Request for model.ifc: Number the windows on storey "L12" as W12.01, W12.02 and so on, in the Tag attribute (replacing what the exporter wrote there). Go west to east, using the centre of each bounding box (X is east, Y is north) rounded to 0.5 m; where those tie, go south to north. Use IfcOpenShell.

First a look at what the model holds.

```python
import ifcopenshell
import ifcopenshell.util.element
import ifcopenshell.util.placement

model = ifcopenshell.open("model.ifc")
print(model.schema)
storey = next(s for s in model.by_type("IfcBuildingStorey") if s.Name == "L12")
windows = [e for e in ifcopenshell.util.element.get_decomposition(storey) if e.is_a("IfcWindow")]
for e in sorted(windows, key=lambda e: e.id()):
    origin = ifcopenshell.util.placement.get_local_placement(e.ObjectPlacement)[:3, 3]
    print(e.id(), e.Tag, e.Name, origin.round(2) + 0.0, sep=" | ")
```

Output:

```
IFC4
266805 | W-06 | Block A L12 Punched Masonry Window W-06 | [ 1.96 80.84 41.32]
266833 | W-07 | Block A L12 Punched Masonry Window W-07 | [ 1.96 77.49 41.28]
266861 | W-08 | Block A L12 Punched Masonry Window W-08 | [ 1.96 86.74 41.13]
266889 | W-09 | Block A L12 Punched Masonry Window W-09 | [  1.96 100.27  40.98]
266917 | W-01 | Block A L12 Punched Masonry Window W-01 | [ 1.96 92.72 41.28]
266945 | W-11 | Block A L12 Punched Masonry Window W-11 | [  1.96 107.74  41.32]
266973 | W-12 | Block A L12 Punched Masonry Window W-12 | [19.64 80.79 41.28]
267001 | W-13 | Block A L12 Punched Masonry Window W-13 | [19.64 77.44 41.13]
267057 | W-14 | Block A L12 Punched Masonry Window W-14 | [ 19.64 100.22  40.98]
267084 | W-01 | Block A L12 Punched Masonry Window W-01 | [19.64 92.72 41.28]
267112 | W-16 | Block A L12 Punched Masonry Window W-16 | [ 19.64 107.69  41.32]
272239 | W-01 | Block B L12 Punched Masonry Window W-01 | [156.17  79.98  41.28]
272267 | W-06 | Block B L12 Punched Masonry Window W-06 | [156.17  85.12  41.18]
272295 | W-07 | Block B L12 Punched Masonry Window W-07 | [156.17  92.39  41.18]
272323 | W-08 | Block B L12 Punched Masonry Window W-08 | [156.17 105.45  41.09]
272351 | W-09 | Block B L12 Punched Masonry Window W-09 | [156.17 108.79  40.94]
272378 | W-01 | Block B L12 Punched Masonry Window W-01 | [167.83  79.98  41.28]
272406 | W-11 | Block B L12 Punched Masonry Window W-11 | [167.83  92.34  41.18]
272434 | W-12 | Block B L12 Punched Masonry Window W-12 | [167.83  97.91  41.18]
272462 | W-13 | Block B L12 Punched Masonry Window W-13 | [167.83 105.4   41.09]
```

```python
import ifcopenshell
import ifcopenshell.geom
import ifcopenshell.util.element
import ifcopenshell.util.shape

model = ifcopenshell.open("model.ifc")
settings = ifcopenshell.geom.settings()
settings.set("use-world-coords", True)


def centre(element):
    shape = ifcopenshell.geom.create_shape(settings, element)
    return ifcopenshell.util.shape.get_bbox_centroid(shape.geometry)


storey = next(s for s in model.by_type("IfcBuildingStorey") if s.Name == "L12")
windows = [e for e in ifcopenshell.util.element.get_decomposition(storey) if e.is_a("IfcWindow")]

# Insertion points can sit at a corner or the storey origin, so sort by the geometry (in metres).
centres = {e: centre(e) for e in windows}
windows.sort(key=lambda e: (round(centres[e][0] / 0.5), centres[e][1]))

for i, e in enumerate(windows, start=1):
    number = f"W12.{i:02d}"
    e.Tag = number
    print(e.id(), number)

model.write("model_rev.ifc")
```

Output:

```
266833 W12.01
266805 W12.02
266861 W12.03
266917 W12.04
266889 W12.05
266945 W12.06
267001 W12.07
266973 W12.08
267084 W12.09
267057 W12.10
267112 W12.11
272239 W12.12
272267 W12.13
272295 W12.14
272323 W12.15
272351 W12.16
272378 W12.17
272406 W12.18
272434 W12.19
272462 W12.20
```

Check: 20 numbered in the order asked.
